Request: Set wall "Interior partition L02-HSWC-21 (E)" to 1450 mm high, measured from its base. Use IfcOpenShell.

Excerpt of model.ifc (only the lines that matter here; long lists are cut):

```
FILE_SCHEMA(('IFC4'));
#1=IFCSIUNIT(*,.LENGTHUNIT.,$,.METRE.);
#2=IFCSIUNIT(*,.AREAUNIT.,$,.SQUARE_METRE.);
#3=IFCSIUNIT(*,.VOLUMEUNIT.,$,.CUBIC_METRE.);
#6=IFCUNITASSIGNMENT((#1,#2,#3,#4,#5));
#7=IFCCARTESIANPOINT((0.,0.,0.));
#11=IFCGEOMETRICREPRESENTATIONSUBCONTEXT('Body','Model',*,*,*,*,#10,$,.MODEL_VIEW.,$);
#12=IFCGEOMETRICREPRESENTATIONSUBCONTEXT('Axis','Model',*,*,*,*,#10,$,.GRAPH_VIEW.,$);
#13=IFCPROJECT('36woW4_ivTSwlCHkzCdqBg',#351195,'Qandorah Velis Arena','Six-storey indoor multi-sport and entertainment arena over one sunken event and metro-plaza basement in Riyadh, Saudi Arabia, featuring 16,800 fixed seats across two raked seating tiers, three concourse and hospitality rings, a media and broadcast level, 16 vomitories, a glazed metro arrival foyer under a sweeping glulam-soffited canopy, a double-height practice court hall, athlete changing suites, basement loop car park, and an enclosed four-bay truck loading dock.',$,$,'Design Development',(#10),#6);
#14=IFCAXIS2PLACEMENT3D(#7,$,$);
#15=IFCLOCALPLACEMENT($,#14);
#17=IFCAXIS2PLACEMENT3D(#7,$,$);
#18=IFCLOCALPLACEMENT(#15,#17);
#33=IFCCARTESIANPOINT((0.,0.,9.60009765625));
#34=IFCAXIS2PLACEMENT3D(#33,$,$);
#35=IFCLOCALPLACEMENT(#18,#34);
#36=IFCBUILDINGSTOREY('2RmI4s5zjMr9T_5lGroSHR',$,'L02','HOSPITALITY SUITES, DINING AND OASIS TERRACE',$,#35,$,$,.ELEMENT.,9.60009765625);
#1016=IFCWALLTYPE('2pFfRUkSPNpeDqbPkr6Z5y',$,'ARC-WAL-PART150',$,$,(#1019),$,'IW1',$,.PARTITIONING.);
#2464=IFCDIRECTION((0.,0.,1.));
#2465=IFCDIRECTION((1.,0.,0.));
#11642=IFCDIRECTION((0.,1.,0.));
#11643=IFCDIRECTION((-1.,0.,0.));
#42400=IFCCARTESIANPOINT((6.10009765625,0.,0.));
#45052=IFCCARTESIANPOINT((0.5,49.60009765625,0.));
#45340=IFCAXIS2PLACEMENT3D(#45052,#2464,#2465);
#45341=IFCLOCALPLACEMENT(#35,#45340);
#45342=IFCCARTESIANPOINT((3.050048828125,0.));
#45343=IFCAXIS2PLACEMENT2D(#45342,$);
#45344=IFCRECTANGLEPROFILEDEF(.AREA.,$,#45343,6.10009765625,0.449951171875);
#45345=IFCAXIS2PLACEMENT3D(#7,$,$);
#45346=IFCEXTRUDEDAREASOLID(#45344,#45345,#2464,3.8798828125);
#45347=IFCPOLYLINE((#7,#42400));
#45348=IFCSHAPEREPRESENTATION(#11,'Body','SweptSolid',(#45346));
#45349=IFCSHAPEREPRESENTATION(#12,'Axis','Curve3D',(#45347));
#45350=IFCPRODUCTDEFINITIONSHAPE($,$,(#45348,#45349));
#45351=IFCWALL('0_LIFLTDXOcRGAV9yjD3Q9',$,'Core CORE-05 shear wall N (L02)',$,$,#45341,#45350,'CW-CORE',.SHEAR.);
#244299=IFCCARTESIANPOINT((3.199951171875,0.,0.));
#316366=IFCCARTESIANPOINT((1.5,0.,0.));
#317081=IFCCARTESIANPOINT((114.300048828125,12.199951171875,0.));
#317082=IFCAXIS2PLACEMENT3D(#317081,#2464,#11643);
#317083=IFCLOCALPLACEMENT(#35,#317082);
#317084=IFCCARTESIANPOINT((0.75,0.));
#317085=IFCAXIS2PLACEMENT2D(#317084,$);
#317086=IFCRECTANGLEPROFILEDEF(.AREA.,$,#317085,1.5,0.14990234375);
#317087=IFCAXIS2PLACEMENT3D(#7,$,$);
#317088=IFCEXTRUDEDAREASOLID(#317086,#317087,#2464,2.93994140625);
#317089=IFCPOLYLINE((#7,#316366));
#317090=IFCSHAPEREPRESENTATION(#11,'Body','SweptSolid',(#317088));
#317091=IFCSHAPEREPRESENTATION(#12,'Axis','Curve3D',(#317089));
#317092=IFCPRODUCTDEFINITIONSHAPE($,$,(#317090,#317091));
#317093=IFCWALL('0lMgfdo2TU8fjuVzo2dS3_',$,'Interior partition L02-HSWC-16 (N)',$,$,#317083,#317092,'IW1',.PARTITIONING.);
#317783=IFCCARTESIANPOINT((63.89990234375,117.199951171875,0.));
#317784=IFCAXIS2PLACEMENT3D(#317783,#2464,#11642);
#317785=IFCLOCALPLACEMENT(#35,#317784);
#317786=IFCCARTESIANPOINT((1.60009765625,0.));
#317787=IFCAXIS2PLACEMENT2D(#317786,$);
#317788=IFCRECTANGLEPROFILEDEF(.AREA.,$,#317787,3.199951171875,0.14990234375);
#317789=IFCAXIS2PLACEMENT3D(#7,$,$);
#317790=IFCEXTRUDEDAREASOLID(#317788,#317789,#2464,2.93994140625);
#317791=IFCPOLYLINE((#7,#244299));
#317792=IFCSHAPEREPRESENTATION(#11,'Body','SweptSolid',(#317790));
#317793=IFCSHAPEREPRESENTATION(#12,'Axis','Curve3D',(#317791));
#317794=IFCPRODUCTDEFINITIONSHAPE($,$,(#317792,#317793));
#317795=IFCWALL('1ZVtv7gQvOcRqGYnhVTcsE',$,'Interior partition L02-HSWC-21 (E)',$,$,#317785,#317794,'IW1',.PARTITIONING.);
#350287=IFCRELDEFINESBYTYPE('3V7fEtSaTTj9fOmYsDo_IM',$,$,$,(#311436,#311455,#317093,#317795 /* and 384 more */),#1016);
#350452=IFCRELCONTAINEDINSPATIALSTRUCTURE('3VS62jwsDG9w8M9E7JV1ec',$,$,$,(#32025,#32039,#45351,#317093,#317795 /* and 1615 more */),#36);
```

```python
import ifcopenshell
import ifcopenshell.geom
import ifcopenshell.util.representation
import ifcopenshell.util.shape

model = ifcopenshell.open("model.ifc")
settings = ifcopenshell.geom.settings()


def volume(element):
    """Net volume in cubic metres, openings subtracted."""
    shape = ifcopenshell.geom.create_shape(settings, element)
    return ifcopenshell.util.shape.get_volume(shape.geometry)


wall = model.by_id(317795)
before = volume(wall)

body = ifcopenshell.util.representation.get_representation(wall, "Model", "Body")
solid = body.Items[0]
old_height = solid.Depth
solid.Depth = 1.45
after = volume(wall)

print(f"height {old_height:g} -> {solid.Depth:g}, volume {before:.3f} -> {after:.3f} m3")

model.write("model_updated.ifc")
```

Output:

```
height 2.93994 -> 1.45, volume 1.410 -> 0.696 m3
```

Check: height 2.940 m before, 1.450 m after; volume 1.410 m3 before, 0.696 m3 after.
